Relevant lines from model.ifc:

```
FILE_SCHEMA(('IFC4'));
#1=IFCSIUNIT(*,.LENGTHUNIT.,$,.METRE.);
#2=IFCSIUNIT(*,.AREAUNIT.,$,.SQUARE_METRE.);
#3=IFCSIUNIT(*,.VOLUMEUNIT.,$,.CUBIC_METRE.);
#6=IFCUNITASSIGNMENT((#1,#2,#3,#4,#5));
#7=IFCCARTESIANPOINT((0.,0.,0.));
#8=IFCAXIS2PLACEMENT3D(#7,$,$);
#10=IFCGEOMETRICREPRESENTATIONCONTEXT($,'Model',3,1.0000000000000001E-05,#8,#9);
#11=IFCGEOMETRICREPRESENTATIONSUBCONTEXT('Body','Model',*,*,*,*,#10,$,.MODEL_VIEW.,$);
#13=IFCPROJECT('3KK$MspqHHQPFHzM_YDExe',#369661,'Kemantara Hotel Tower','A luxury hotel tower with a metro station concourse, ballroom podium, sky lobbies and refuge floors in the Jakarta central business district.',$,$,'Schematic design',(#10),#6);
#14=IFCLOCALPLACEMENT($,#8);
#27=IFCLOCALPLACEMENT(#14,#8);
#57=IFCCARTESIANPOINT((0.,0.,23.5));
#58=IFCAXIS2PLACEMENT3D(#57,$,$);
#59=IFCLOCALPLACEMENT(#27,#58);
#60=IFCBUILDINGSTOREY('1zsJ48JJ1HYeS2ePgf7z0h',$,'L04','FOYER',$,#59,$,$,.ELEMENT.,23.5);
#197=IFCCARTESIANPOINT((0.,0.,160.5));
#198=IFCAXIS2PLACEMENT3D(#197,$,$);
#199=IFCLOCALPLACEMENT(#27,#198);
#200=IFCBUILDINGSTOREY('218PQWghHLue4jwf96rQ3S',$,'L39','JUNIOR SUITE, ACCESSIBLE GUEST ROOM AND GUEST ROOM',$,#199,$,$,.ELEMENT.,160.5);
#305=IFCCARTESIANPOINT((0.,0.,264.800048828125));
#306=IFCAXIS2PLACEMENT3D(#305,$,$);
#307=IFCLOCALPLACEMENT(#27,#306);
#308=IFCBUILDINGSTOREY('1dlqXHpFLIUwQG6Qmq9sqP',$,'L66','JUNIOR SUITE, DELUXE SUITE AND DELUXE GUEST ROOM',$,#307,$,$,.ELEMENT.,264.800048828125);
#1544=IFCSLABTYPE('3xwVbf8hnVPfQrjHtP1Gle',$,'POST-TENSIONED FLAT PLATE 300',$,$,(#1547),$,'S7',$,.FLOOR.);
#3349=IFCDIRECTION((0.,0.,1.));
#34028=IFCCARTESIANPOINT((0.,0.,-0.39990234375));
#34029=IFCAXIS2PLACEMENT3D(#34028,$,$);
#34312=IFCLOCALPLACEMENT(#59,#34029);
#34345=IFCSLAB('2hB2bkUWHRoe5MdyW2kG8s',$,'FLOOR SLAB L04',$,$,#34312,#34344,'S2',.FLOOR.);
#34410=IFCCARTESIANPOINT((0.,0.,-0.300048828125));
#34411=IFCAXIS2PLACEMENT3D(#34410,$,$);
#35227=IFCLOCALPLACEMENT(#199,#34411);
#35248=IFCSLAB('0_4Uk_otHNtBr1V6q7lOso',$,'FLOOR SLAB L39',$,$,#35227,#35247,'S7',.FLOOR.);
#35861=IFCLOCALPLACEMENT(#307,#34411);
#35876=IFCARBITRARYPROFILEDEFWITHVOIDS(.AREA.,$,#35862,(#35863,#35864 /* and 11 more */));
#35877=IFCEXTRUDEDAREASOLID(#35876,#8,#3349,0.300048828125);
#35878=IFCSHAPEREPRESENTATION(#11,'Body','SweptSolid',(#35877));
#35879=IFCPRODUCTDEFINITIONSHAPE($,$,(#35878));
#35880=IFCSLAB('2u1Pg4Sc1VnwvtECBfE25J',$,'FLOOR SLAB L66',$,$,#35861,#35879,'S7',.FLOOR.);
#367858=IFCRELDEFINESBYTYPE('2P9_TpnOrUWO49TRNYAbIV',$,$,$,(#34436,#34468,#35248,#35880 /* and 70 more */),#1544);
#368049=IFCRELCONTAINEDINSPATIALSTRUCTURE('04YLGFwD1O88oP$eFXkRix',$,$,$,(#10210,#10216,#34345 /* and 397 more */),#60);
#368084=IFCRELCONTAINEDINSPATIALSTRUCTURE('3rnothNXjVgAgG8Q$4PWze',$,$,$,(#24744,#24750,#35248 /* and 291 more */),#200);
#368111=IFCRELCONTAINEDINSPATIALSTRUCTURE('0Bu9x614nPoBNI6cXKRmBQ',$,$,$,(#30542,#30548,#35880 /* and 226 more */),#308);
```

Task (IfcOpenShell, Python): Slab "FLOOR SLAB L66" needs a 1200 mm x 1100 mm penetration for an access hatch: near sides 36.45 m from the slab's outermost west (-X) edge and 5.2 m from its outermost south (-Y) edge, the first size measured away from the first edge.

```python
import numpy as np
import ifcopenshell
import ifcopenshell.api.feature
import ifcopenshell.api.geometry
import ifcopenshell.api.root
import ifcopenshell.geom
import ifcopenshell.util.placement
import ifcopenshell.util.representation
import ifcopenshell.util.shape
import ifcopenshell.util.unit

model = ifcopenshell.open("model.ifc")
unit_scale = ifcopenshell.util.unit.calculate_unit_scale(model)
settings = ifcopenshell.geom.settings()


def volume(element):
    """Net volume in cubic metres, openings subtracted."""
    shape = ifcopenshell.geom.create_shape(settings, element)
    return ifcopenshell.util.shape.get_volume(shape.geometry)


slab = model.by_guid("2u1Pg4Sc1VnwvtECBfE25J")
before = volume(slab)

# Extent in the slab's own axes, in metres. The edges named are its -X and -Y sides.
slab_shape = ifcopenshell.geom.create_shape(settings, slab)
vertices = ifcopenshell.util.shape.get_vertices(slab_shape.geometry)
x_min, y_min, bottom = vertices.min(axis=0)
top = vertices[:, 2].max()

opening = ifcopenshell.api.root.create_entity(model, ifc_class="IfcOpeningElement", name="Access hatch opening", predefined_type="OPENING")
context = ifcopenshell.util.representation.get_context(model, "Model", "Body", "MODEL_VIEW")
width, depth = 1.2, 1.1
outline = [(0.0, 0.0), (width, 0.0), (width, depth), (0.0, depth), (0.0, 0.0)]
# Overshoot both faces by 50 mm so the cut is clean.
shape = ifcopenshell.api.geometry.add_slab_representation(
    model, context=context, depth=top - bottom + 0.1, polyline=outline
)
ifcopenshell.api.geometry.assign_representation(model, product=opening, representation=shape)

matrix = ifcopenshell.util.placement.get_local_placement(slab.ObjectPlacement)
matrix[:, 3] = matrix @ np.append(np.array([x_min + 36.45, y_min + 5.2, bottom - 0.05]) / unit_scale, 1.0)
ifcopenshell.api.geometry.edit_object_placement(model, product=opening, matrix=matrix, is_si=False)
ifcopenshell.api.feature.add_feature(model, feature=opening, element=slab)

after = volume(slab)

print(f"slab volume {before:.3f} -> {after:.3f} m3")

model.write("model_updated.ifc")
```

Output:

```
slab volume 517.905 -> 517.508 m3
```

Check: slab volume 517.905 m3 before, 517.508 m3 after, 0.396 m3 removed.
